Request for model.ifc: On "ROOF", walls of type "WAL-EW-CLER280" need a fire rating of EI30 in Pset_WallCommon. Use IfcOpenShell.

First a look at what the model holds.

```python
import ifcopenshell
import ifcopenshell.util.element

model = ifcopenshell.open("model.ifc")
print(model.schema)
storey = next(s for s in model.by_type("IfcBuildingStorey") if s.Name == "ROOF")
walls = [e for e in ifcopenshell.util.element.get_decomposition(storey) if e.is_a("IfcWall")]
seen = {}
for e in walls:
    element_type = ifcopenshell.util.element.get_type(e)
    key = (element_type.Name if element_type != e and element_type else None, ifcopenshell.util.element.get_pset(e, "Pset_WallCommon", "FireRating"))
    seen[key] = seen.get(key, 0) + 1
for (name, value), count in sorted(seen.items(), key=str):
    print(count, "x", name, "|", value)
```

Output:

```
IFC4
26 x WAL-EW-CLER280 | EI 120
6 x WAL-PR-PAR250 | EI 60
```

```python
import ifcopenshell
import ifcopenshell.api.pset
import ifcopenshell.util.element

model = ifcopenshell.open("model.ifc")

storey = next(s for s in model.by_type("IfcBuildingStorey") if s.Name == "ROOF")
walls = [e for e in ifcopenshell.util.element.get_decomposition(storey) if e.is_a("IfcWall")]

count = 0
for e in walls:
    element_type = ifcopenshell.util.element.get_type(e)
    if element_type in (None, e) or element_type.Name != "WAL-EW-CLER280":
        continue
    # add_pset returns the element's existing set when there is one.
    pset = ifcopenshell.api.pset.add_pset(model, product=e, name="Pset_WallCommon")
    ifcopenshell.api.pset.edit_pset(model, pset=pset, properties={"FireRating": "EI30"})
    count += 1

print(count, "walls updated")

model.write("model_rev.ifc")
```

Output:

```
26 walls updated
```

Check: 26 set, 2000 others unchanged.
